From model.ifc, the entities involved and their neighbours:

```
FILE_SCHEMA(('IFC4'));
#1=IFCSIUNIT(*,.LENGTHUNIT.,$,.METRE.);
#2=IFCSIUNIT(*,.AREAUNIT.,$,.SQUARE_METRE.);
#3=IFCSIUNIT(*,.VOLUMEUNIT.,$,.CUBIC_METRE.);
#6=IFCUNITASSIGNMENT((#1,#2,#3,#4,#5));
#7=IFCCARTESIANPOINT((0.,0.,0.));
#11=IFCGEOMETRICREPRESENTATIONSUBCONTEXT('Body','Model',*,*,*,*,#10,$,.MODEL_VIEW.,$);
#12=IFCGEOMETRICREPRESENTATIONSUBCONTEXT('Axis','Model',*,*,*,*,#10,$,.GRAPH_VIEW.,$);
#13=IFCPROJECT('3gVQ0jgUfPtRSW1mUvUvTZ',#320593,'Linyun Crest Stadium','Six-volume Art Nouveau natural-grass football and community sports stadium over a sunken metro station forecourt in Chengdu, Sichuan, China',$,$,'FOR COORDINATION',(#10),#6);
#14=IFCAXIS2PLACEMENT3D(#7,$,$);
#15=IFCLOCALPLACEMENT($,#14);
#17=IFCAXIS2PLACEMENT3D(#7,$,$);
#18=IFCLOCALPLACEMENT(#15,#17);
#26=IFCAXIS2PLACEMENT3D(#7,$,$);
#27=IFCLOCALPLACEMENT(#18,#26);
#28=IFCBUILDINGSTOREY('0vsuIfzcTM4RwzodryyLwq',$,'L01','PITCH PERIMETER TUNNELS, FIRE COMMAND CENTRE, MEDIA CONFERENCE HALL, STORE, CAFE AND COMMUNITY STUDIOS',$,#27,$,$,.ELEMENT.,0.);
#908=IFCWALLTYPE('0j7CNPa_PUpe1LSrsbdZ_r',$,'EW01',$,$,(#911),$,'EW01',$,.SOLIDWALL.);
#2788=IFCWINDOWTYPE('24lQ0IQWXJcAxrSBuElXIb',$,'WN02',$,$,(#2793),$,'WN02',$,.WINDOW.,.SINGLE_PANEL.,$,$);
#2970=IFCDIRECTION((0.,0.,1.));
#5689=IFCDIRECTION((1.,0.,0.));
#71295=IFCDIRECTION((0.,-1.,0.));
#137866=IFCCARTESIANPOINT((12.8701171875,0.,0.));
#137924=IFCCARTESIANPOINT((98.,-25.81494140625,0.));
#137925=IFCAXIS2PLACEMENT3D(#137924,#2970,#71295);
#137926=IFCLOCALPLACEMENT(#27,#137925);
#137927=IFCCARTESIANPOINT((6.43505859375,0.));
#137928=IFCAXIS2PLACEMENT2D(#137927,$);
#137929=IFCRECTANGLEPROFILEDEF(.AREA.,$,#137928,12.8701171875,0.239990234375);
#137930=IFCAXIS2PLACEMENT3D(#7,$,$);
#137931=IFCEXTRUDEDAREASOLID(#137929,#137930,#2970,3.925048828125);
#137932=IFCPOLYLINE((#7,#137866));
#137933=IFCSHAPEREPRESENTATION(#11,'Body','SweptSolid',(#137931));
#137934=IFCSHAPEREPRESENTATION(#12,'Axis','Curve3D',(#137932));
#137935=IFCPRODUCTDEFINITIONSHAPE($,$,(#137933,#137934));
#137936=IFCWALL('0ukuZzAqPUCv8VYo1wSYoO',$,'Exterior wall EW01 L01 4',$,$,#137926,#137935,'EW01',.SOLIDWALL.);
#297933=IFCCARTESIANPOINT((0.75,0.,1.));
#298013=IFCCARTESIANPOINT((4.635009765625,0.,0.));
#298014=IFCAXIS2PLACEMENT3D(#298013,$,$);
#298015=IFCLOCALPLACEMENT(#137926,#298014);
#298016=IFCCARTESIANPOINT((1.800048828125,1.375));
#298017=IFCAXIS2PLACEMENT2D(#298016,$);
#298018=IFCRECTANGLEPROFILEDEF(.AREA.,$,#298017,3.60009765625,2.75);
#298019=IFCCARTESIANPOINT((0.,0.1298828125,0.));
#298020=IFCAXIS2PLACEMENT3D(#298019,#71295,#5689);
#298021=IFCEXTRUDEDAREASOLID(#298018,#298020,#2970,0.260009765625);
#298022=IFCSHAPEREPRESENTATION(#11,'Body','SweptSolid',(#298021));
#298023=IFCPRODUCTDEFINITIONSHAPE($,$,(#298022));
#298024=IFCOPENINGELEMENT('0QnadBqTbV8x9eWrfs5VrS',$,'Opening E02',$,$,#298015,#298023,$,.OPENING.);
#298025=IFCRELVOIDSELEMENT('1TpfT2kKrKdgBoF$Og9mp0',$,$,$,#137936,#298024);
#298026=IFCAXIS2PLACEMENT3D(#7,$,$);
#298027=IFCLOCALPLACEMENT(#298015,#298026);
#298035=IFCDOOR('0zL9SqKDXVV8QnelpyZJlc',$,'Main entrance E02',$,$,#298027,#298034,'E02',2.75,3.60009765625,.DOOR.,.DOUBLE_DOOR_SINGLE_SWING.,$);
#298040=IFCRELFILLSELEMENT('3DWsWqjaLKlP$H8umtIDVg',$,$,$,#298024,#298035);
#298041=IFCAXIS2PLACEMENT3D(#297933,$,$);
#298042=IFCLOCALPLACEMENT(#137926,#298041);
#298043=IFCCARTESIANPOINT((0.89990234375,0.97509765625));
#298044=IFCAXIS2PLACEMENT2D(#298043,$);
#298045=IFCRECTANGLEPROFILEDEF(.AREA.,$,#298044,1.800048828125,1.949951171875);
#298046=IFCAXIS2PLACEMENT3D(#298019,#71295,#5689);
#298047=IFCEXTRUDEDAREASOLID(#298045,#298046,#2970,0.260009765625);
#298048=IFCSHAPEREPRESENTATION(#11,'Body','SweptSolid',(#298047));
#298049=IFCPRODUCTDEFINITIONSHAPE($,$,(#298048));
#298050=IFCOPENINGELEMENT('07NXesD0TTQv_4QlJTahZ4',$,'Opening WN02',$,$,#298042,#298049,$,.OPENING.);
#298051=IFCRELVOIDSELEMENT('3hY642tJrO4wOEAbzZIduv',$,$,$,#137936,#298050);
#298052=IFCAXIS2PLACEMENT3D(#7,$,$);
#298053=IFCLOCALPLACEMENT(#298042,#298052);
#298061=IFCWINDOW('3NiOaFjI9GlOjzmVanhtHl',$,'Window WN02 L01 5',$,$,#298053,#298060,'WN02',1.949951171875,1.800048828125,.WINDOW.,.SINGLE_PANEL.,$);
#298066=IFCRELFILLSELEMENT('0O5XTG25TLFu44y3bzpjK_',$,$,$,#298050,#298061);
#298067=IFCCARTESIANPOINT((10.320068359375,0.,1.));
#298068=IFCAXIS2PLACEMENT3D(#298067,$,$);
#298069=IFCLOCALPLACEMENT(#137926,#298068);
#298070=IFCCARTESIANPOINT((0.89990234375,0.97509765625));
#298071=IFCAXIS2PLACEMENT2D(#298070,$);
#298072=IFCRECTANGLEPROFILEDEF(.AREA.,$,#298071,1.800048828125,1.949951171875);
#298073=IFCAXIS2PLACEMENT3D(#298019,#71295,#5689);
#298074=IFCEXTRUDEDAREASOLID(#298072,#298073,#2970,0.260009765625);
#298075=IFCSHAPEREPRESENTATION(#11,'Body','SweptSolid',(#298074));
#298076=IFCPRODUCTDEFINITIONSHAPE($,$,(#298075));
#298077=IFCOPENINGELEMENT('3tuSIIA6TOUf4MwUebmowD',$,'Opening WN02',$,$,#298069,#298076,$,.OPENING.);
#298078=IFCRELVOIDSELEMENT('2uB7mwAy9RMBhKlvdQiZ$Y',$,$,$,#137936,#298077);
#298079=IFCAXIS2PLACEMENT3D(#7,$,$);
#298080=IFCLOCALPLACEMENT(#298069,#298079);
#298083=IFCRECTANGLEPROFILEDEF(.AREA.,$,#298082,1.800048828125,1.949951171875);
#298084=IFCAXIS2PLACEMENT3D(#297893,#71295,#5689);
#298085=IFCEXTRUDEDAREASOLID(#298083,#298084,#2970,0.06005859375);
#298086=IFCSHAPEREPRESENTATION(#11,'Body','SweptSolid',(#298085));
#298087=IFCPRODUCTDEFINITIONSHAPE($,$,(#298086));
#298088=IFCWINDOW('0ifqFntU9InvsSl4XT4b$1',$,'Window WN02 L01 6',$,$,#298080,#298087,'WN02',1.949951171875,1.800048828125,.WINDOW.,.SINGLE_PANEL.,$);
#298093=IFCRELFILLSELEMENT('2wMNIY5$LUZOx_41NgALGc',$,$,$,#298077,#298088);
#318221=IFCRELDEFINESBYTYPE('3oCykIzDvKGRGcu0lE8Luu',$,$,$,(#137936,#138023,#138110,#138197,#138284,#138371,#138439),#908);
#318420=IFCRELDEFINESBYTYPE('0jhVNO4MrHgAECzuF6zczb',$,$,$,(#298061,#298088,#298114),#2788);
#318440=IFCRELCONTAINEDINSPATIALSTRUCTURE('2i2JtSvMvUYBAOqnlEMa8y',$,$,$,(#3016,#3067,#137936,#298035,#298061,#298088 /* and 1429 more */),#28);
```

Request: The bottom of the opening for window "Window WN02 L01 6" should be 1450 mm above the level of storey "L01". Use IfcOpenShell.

```python
import numpy as np
import ifcopenshell
import ifcopenshell.api.geometry
import ifcopenshell.geom
import ifcopenshell.util.element
import ifcopenshell.util.placement
import ifcopenshell.util.shape
import ifcopenshell.util.unit

model = ifcopenshell.open("model.ifc")
unit_scale = ifcopenshell.util.unit.calculate_unit_scale(model)

window = model.by_id(298088)
opening = window.FillsVoids[0].RelatingOpeningElement
storey = ifcopenshell.util.element.get_container(window, ifc_class="IfcBuildingStorey")
level = ifcopenshell.util.placement.get_local_placement(storey.ObjectPlacement)[2, 3]

# The opening's origin need not be at the sill, so measure its lowest point.
shape = ifcopenshell.geom.create_shape(ifcopenshell.geom.settings(), opening)
bottom = ifcopenshell.util.shape.get_shape_bottom_elevation(shape, shape.geometry) / unit_scale
dz = level + 1.45 / unit_scale - bottom

shift = np.array([0.0, 0.0, dz])
# The window is placed relative to its opening, so it follows when the opening moves.
matrix = ifcopenshell.util.placement.get_local_placement(opening.ObjectPlacement)
matrix[:3, 3] += shift
ifcopenshell.api.geometry.edit_object_placement(
    model, product=opening, matrix=matrix, is_si=False, should_transform_children=True
)

print(f"moved by {dz * unit_scale:+.3f} m")

model.write("model-out.ifc")
```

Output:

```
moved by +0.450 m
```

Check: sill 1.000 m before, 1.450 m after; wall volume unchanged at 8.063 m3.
